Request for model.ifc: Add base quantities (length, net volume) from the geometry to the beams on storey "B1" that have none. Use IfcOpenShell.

First a look at what the model holds.

```python
import ifcopenshell
import ifcopenshell.util.element
import ifcopenshell.util.unit

model = ifcopenshell.open("model.ifc")
print(model.schema)
for unit_type in ("LENGTHUNIT", "AREAUNIT", "VOLUMEUNIT"):
    print(unit_type, ifcopenshell.util.unit.calculate_unit_scale(model, unit_type))
storey = next(s for s in model.by_type("IfcBuildingStorey") if s.Name == "B1")
beams = [e for e in ifcopenshell.util.element.get_decomposition(storey) if e.is_a("IfcBeam")]
for e in sorted(beams, key=lambda e: e.id()):
    print(e.id(), e.is_a(), e.Name, list(ifcopenshell.util.element.get_psets(e, qtos_only=True)), sep=" | ")
```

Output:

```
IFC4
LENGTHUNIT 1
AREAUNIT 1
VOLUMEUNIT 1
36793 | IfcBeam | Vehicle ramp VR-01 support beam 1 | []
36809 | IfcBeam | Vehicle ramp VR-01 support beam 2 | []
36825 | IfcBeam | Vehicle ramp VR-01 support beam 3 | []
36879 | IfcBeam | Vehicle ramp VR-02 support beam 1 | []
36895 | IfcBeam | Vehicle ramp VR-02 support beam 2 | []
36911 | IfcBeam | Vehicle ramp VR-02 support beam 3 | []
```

```python
import ifcopenshell
import ifcopenshell.api.pset
import ifcopenshell.geom
import ifcopenshell.util.element
import ifcopenshell.util.shape
import ifcopenshell.util.unit

model = ifcopenshell.open("model.ifc")
unit_scale = ifcopenshell.util.unit.calculate_unit_scale(model)
volume_scale = ifcopenshell.util.unit.calculate_unit_scale(model, "VOLUMEUNIT")
settings = ifcopenshell.geom.settings()

storey = next(s for s in model.by_type("IfcBuildingStorey") if s.Name == "B1")
beams = [e for e in ifcopenshell.util.element.get_decomposition(storey) if e.is_a("IfcBeam")]

for e in sorted(beams, key=lambda e: e.id()):
    if ifcopenshell.util.element.get_psets(e, qtos_only=True, should_inherit=False):
        continue
    # Geometry comes back in metres, in the element's own axes.
    shape = ifcopenshell.geom.create_shape(settings, e)
    values = {
        "Length": ifcopenshell.util.shape.get_max_xyz(shape.geometry) / unit_scale,
        "NetVolume": ifcopenshell.util.shape.get_volume(shape.geometry) / volume_scale,
    }
    qto = ifcopenshell.api.pset.add_qto(model, product=e, name="Qto_BeamBaseQuantities")
    ifcopenshell.api.pset.edit_qto(model, qto=qto, properties=values)
    print(e.id(), {k: round(v, 3) for k, v in values.items()})

model.write("model_v2.ifc")
```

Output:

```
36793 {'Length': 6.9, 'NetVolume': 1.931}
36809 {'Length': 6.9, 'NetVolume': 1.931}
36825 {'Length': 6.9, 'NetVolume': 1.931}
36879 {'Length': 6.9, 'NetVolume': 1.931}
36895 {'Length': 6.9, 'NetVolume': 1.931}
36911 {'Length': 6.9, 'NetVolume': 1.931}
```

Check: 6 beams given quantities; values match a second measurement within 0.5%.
